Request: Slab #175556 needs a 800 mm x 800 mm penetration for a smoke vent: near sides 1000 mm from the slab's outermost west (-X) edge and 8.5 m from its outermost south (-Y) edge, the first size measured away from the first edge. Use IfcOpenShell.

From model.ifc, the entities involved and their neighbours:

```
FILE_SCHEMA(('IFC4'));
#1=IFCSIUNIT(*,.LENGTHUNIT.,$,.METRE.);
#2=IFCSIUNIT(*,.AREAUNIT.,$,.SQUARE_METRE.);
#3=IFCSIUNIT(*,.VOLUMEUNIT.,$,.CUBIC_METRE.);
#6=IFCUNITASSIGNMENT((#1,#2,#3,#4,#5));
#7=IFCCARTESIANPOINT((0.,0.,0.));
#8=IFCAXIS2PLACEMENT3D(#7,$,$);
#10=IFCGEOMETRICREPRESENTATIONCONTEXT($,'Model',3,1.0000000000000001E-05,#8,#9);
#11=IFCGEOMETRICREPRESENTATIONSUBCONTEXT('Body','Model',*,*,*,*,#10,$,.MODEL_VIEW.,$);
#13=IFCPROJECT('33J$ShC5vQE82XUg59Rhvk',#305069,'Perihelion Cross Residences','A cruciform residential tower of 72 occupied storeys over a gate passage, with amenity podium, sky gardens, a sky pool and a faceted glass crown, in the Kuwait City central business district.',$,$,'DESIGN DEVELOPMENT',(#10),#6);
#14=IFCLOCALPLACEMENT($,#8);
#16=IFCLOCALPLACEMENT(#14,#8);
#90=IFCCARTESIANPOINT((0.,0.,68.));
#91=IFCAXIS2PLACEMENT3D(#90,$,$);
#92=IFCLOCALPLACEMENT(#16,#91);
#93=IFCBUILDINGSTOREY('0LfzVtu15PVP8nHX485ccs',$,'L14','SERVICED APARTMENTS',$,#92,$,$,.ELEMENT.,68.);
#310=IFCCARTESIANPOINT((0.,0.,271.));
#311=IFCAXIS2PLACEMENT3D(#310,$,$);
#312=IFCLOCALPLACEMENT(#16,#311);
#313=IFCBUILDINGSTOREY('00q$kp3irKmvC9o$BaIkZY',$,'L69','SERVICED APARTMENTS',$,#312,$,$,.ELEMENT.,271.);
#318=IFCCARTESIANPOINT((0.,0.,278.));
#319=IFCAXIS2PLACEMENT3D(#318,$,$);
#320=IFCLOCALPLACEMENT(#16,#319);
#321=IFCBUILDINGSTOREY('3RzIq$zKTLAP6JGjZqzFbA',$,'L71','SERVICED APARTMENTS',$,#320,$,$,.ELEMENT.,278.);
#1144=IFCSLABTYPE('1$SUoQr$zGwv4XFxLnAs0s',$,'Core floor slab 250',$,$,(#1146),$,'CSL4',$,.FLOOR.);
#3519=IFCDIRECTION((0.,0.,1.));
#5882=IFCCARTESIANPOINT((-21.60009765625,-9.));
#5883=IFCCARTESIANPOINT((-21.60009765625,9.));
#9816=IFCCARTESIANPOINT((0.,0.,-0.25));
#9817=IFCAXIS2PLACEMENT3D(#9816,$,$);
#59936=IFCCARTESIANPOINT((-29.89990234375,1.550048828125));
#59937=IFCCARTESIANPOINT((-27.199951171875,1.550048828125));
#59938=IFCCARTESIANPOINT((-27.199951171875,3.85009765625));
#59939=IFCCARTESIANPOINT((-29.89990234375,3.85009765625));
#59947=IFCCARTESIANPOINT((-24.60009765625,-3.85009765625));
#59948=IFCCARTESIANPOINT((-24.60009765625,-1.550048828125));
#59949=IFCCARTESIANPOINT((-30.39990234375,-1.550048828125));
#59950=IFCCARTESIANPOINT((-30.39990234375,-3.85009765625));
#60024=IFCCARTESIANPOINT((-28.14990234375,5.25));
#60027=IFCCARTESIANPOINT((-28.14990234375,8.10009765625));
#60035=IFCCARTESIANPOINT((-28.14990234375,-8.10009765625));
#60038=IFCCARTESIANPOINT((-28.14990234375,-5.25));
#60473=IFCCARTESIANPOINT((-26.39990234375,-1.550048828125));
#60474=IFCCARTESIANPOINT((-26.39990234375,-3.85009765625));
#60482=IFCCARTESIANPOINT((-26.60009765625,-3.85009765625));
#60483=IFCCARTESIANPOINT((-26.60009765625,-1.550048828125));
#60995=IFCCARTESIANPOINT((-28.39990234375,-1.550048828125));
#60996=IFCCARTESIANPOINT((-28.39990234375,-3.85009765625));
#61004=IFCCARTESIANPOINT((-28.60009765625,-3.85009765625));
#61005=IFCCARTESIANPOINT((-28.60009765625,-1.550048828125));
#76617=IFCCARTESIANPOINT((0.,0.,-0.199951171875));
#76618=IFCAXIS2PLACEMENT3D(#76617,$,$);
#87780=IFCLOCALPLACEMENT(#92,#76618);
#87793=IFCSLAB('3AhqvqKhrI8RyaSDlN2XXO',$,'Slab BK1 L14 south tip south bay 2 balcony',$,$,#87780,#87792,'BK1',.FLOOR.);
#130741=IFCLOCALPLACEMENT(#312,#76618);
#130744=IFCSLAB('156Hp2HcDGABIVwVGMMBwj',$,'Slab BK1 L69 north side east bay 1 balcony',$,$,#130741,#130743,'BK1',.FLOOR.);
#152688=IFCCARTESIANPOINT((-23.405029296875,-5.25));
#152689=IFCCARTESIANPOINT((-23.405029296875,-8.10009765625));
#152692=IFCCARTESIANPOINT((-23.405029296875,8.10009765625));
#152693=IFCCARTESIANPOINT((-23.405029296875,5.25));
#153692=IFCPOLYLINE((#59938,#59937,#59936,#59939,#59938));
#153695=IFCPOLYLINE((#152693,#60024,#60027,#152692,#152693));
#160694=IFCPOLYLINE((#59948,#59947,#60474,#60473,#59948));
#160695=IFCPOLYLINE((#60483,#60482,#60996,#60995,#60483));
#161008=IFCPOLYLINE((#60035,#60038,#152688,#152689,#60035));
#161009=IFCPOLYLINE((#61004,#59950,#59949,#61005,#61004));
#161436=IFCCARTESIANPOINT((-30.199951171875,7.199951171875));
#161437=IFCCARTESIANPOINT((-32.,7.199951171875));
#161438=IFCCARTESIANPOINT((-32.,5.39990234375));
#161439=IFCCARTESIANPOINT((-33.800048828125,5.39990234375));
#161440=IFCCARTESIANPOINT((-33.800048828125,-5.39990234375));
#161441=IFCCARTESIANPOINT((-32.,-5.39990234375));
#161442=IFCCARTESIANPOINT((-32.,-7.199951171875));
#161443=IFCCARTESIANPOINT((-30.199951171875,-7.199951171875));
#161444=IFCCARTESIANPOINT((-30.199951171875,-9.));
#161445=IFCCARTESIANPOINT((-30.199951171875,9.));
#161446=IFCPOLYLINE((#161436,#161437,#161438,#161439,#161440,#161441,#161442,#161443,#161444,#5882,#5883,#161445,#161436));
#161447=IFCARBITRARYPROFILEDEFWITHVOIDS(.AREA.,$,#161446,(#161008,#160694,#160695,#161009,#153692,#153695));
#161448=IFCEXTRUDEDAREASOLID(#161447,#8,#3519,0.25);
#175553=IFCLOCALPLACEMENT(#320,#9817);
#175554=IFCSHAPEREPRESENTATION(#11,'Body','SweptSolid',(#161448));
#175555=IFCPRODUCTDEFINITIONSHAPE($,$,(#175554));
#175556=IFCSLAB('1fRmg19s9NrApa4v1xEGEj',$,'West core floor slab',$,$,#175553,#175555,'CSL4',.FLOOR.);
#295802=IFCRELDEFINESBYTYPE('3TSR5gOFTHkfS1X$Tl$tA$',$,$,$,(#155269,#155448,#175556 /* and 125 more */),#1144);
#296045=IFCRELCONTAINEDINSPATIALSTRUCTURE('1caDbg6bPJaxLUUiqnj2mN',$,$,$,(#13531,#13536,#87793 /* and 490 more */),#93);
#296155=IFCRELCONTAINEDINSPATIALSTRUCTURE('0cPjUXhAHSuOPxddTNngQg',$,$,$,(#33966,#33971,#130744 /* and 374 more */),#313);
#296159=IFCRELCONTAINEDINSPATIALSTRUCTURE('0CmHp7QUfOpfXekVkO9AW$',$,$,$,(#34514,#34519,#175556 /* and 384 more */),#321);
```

```python
import numpy as np
import ifcopenshell
import ifcopenshell.api.feature
import ifcopenshell.api.geometry
import ifcopenshell.api.root
import ifcopenshell.geom
import ifcopenshell.util.placement
import ifcopenshell.util.representation
import ifcopenshell.util.shape
import ifcopenshell.util.unit

model = ifcopenshell.open("model.ifc")
unit_scale = ifcopenshell.util.unit.calculate_unit_scale(model)
settings = ifcopenshell.geom.settings()


def volume(element):
    """Net volume in cubic metres, openings subtracted."""
    shape = ifcopenshell.geom.create_shape(settings, element)
    return ifcopenshell.util.shape.get_volume(shape.geometry)


slab = model.by_guid("1fRmg19s9NrApa4v1xEGEj")
before = volume(slab)

# Extent in the slab's own axes, in metres. The edges named are its -X and -Y sides.
slab_shape = ifcopenshell.geom.create_shape(settings, slab)
vertices = ifcopenshell.util.shape.get_vertices(slab_shape.geometry)
x_min, y_min, bottom = vertices.min(axis=0)
top = vertices[:, 2].max()

opening = ifcopenshell.api.root.create_entity(model, ifc_class="IfcOpeningElement", name="Smoke vent opening", predefined_type="OPENING")
context = ifcopenshell.util.representation.get_context(model, "Model", "Body", "MODEL_VIEW")
width, depth = 0.8, 0.8
outline = [(0.0, 0.0), (width, 0.0), (width, depth), (0.0, depth), (0.0, 0.0)]
# Overshoot both faces by 50 mm so the cut is clean.
shape = ifcopenshell.api.geometry.add_slab_representation(
    model, context=context, depth=top - bottom + 0.1, polyline=outline
)
ifcopenshell.api.geometry.assign_representation(model, product=opening, representation=shape)

matrix = ifcopenshell.util.placement.get_local_placement(slab.ObjectPlacement)
matrix[:, 3] = matrix @ np.append(np.array([x_min + 1, y_min + 8.5, bottom - 0.05]) / unit_scale, 1.0)
ifcopenshell.api.geometry.edit_object_placement(model, product=opening, matrix=matrix, is_si=False)
ifcopenshell.api.feature.add_feature(model, feature=opening, element=slab)

after = volume(slab)

print(f"slab volume {before:.3f} -> {after:.3f} m3")

model.write("model_rev.ifc")
```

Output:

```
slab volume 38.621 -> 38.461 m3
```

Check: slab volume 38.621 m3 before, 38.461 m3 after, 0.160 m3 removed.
